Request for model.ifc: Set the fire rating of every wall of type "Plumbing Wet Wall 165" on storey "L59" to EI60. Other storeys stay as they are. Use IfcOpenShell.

First a look at what the model holds.

```python
import ifcopenshell
import ifcopenshell.util.element

model = ifcopenshell.open("model.ifc")
print(model.schema)
storey = next(s for s in model.by_type("IfcBuildingStorey") if s.Name == "L59")
walls = [e for e in ifcopenshell.util.element.get_decomposition(storey) if e.is_a("IfcWall")]
seen = {}
for e in walls:
    element_type = ifcopenshell.util.element.get_type(e)
    key = (element_type.Name if element_type != e and element_type else None, ifcopenshell.util.element.get_pset(e, "Pset_WallCommon", "FireRating"))
    seen[key] = seen.get(key, 0) + 1
for (name, value), count in sorted(seen.items(), key=str):
    print(count, "x", name, "|", value)
```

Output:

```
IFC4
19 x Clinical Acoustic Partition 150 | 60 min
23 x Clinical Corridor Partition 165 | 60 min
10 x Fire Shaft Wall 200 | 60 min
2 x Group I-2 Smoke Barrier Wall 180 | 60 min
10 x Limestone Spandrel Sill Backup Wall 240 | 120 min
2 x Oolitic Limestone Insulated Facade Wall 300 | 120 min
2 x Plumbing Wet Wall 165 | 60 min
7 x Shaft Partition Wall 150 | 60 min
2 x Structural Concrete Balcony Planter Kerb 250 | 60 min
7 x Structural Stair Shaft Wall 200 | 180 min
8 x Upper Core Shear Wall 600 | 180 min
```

```python
import ifcopenshell
import ifcopenshell.api.pset
import ifcopenshell.util.element

model = ifcopenshell.open("model.ifc")

storey = next(s for s in model.by_type("IfcBuildingStorey") if s.Name == "L59")
walls = [e for e in ifcopenshell.util.element.get_decomposition(storey) if e.is_a("IfcWall")]

count = 0
for e in walls:
    element_type = ifcopenshell.util.element.get_type(e)
    if element_type in (None, e) or element_type.Name != "Plumbing Wet Wall 165":
        continue
    found = ifcopenshell.util.element.get_pset(e, "Pset_WallCommon", should_inherit=False)
    if found:
        pset = model.by_id(found["id"])
        if len(ifcopenshell.util.element.get_elements_by_pset(pset)) > 1:
            pset = ifcopenshell.api.pset.unshare_pset(model, products=[e], pset=pset)[0]
    else:
        pset = ifcopenshell.api.pset.add_pset(model, product=e, name="Pset_WallCommon")
    ifcopenshell.api.pset.edit_pset(model, pset=pset, properties={"FireRating": "EI60"})
    count += 1

print(count, "walls updated")

model.write("model_edited.ifc")
```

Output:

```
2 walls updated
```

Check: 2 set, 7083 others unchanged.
